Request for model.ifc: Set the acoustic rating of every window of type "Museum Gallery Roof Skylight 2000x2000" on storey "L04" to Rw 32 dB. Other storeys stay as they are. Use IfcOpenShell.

First a look at what the model holds.

```python
import ifcopenshell
import ifcopenshell.util.element

model = ifcopenshell.open("model.ifc")
print(model.schema)
storey = next(s for s in model.by_type("IfcBuildingStorey") if s.Name == "L04")
windows = [e for e in ifcopenshell.util.element.get_decomposition(storey) if e.is_a("IfcWindow")]
seen = {}
for e in windows:
    element_type = ifcopenshell.util.element.get_type(e)
    key = (element_type.Name if element_type != e and element_type else None, ifcopenshell.util.element.get_pset(e, "Pset_WindowCommon", "AcousticRating"))
    seen[key] = seen.get(key, 0) + 1
for (name, value), count in sorted(seen.items(), key=str):
    print(count, "x", name, "|", value)
```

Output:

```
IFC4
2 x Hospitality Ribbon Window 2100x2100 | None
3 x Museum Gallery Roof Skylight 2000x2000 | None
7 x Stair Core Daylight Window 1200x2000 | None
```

```python
import ifcopenshell
import ifcopenshell.api.pset
import ifcopenshell.util.element

model = ifcopenshell.open("model.ifc")

storey = next(s for s in model.by_type("IfcBuildingStorey") if s.Name == "L04")
windows = [e for e in ifcopenshell.util.element.get_decomposition(storey) if e.is_a("IfcWindow")]

count = 0
for e in windows:
    element_type = ifcopenshell.util.element.get_type(e)
    if element_type in (None, e) or element_type.Name != "Museum Gallery Roof Skylight 2000x2000":
        continue
    # add_pset returns the element's existing set when there is one.
    pset = ifcopenshell.api.pset.add_pset(model, product=e, name="Pset_WindowCommon")
    ifcopenshell.api.pset.edit_pset(model, pset=pset, properties={"AcousticRating": "Rw 32 dB"})
    count += 1

print(count, "windows updated")

model.write("model-out.ifc")
```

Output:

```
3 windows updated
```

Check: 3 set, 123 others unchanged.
